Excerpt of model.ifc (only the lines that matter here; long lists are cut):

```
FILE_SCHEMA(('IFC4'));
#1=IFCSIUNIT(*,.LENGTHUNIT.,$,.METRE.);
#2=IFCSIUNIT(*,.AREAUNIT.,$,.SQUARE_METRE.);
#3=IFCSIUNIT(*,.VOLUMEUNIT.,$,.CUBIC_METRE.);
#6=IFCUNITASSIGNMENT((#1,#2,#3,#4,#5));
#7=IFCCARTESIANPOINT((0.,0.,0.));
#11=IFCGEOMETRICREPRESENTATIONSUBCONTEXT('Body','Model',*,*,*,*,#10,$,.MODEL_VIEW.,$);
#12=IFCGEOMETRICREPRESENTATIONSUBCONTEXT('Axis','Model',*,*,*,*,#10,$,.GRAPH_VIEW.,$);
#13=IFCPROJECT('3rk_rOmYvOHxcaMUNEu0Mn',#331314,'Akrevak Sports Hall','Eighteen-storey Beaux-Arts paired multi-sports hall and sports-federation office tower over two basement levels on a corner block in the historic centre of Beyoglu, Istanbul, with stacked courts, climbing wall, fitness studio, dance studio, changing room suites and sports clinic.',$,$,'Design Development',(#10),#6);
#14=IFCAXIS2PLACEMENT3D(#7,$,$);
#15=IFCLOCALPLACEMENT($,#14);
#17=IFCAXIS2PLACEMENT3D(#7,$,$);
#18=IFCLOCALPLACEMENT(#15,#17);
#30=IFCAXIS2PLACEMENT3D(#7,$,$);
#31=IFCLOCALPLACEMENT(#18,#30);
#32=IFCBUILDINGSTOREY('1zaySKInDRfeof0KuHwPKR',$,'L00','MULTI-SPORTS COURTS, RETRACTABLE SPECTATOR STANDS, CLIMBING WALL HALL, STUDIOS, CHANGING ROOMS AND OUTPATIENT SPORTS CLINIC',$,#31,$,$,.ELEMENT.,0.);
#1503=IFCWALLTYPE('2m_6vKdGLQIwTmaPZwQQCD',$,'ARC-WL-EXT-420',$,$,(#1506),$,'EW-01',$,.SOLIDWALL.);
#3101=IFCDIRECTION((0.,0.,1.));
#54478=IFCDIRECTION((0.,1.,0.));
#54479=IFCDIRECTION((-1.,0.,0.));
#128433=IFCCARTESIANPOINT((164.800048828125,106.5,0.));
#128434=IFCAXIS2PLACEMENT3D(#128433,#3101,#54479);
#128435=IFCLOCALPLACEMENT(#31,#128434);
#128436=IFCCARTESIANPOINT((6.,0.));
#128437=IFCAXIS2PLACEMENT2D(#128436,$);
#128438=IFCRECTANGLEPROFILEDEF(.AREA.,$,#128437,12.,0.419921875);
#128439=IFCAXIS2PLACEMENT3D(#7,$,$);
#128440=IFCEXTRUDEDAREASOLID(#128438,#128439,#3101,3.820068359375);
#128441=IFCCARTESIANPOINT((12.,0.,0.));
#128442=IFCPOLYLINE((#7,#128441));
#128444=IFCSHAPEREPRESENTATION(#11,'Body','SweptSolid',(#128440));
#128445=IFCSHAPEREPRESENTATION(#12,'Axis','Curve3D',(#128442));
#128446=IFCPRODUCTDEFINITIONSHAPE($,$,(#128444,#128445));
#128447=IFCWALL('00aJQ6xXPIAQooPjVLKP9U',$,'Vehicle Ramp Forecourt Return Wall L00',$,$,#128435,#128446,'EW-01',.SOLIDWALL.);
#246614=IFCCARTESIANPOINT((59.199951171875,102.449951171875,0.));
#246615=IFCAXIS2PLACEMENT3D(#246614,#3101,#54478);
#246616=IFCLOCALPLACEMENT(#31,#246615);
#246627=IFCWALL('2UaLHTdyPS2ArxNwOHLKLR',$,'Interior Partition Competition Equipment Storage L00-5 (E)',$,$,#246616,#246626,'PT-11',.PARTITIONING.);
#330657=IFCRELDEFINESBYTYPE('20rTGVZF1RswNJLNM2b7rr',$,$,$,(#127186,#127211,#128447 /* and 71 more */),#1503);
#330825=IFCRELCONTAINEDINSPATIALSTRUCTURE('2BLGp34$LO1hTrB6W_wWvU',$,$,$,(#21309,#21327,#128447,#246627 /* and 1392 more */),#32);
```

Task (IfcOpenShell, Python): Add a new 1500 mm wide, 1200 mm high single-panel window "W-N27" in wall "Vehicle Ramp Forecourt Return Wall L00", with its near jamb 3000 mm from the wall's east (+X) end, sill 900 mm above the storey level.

```python
import numpy as np
import ifcopenshell
import ifcopenshell.api.feature
import ifcopenshell.api.geometry
import ifcopenshell.api.root
import ifcopenshell.api.spatial
import ifcopenshell.geom
import ifcopenshell.util.element
import ifcopenshell.util.placement
import ifcopenshell.util.representation
import ifcopenshell.util.shape
import ifcopenshell.util.unit

model = ifcopenshell.open("model.ifc")
unit_scale = ifcopenshell.util.unit.calculate_unit_scale(model)
settings = ifcopenshell.geom.settings()


def volume(element):
    """Net volume in cubic metres, openings subtracted."""
    shape = ifcopenshell.geom.create_shape(settings, element)
    return ifcopenshell.util.shape.get_volume(shape.geometry)


wall = model.by_guid("00aJQ6xXPIAQooPjVLKP9U")
storey = ifcopenshell.util.element.get_container(wall, ifc_class="IfcBuildingStorey")
context = ifcopenshell.util.representation.get_context(model, "Model", "Body", "MODEL_VIEW")
before = volume(wall)

width, height, from_end, sill = 1.5, 1.2, 3, 0.9  # metres

# The wall runs along its own X axis, and the end named is its -X end.
wall_shape = ifcopenshell.geom.create_shape(settings, wall)
x, y, z = ifcopenshell.util.shape.get_vertices(wall_shape.geometry).T
start = x.min() + from_end
face, thickness = float(y.min()), float(y.max() - y.min())
wall_matrix = ifcopenshell.util.placement.get_local_placement(wall.ObjectPlacement)
level = ifcopenshell.util.placement.get_local_placement(storey.ObjectPlacement)[2, 3]


def in_wall(x, y):
    """Placement at x, y metres in the wall's axes, at sill height."""
    matrix = wall_matrix.copy()
    matrix[:, 3] = wall_matrix @ np.array([x / unit_scale, y / unit_scale, 0.0, 1.0])
    matrix[2, 3] = level + sill / unit_scale
    return matrix


# Opening: a box that overshoots both wall faces by 50 mm.
opening = ifcopenshell.api.root.create_entity(model, ifc_class="IfcOpeningElement", predefined_type="OPENING")
box = ifcopenshell.api.geometry.add_wall_representation(
    model, context=context, length=width, height=height, thickness=thickness + 0.1
)
ifcopenshell.api.geometry.assign_representation(model, product=opening, representation=box)
ifcopenshell.api.geometry.edit_object_placement(model, product=opening, matrix=in_wall(start, face - 0.05), is_si=False)
ifcopenshell.api.feature.add_feature(model, feature=opening, element=wall)

window = ifcopenshell.api.root.create_entity(model, ifc_class="IfcWindow", name="W-N27", predefined_type="WINDOW")
window.OverallWidth, window.OverallHeight = width / unit_scale, height / unit_scale
window.PartitioningType = "SINGLE_PANEL"
body = ifcopenshell.api.geometry.add_window_representation(
    model,
    context=context,
    overall_width=window.OverallWidth,
    overall_height=window.OverallHeight,
    partition_type="SINGLE_PANEL",
)
ifcopenshell.api.geometry.assign_representation(model, product=window, representation=body)
ifcopenshell.api.spatial.assign_container(model, products=[window], relating_structure=storey)
ifcopenshell.api.feature.add_filling(model, opening=opening, element=window)

# Centre the window in the wall's thickness.
ifcopenshell.api.geometry.edit_object_placement(model, product=window, matrix=in_wall(start, face), is_si=False)
window_shape = ifcopenshell.geom.create_shape(settings, window)
depth = ifcopenshell.util.shape.get_vertices(window_shape.geometry)[:, 1]
offset = face + thickness / 2 - (depth.min() + depth.max()) / 2
ifcopenshell.api.geometry.edit_object_placement(model, product=window, matrix=in_wall(start, offset), is_si=False)

after = volume(wall)

print(f"wall volume {before:.3f} -> {after:.3f} m3")

model.write("model_rev.ifc")
```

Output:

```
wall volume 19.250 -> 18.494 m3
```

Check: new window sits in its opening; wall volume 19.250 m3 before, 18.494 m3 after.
